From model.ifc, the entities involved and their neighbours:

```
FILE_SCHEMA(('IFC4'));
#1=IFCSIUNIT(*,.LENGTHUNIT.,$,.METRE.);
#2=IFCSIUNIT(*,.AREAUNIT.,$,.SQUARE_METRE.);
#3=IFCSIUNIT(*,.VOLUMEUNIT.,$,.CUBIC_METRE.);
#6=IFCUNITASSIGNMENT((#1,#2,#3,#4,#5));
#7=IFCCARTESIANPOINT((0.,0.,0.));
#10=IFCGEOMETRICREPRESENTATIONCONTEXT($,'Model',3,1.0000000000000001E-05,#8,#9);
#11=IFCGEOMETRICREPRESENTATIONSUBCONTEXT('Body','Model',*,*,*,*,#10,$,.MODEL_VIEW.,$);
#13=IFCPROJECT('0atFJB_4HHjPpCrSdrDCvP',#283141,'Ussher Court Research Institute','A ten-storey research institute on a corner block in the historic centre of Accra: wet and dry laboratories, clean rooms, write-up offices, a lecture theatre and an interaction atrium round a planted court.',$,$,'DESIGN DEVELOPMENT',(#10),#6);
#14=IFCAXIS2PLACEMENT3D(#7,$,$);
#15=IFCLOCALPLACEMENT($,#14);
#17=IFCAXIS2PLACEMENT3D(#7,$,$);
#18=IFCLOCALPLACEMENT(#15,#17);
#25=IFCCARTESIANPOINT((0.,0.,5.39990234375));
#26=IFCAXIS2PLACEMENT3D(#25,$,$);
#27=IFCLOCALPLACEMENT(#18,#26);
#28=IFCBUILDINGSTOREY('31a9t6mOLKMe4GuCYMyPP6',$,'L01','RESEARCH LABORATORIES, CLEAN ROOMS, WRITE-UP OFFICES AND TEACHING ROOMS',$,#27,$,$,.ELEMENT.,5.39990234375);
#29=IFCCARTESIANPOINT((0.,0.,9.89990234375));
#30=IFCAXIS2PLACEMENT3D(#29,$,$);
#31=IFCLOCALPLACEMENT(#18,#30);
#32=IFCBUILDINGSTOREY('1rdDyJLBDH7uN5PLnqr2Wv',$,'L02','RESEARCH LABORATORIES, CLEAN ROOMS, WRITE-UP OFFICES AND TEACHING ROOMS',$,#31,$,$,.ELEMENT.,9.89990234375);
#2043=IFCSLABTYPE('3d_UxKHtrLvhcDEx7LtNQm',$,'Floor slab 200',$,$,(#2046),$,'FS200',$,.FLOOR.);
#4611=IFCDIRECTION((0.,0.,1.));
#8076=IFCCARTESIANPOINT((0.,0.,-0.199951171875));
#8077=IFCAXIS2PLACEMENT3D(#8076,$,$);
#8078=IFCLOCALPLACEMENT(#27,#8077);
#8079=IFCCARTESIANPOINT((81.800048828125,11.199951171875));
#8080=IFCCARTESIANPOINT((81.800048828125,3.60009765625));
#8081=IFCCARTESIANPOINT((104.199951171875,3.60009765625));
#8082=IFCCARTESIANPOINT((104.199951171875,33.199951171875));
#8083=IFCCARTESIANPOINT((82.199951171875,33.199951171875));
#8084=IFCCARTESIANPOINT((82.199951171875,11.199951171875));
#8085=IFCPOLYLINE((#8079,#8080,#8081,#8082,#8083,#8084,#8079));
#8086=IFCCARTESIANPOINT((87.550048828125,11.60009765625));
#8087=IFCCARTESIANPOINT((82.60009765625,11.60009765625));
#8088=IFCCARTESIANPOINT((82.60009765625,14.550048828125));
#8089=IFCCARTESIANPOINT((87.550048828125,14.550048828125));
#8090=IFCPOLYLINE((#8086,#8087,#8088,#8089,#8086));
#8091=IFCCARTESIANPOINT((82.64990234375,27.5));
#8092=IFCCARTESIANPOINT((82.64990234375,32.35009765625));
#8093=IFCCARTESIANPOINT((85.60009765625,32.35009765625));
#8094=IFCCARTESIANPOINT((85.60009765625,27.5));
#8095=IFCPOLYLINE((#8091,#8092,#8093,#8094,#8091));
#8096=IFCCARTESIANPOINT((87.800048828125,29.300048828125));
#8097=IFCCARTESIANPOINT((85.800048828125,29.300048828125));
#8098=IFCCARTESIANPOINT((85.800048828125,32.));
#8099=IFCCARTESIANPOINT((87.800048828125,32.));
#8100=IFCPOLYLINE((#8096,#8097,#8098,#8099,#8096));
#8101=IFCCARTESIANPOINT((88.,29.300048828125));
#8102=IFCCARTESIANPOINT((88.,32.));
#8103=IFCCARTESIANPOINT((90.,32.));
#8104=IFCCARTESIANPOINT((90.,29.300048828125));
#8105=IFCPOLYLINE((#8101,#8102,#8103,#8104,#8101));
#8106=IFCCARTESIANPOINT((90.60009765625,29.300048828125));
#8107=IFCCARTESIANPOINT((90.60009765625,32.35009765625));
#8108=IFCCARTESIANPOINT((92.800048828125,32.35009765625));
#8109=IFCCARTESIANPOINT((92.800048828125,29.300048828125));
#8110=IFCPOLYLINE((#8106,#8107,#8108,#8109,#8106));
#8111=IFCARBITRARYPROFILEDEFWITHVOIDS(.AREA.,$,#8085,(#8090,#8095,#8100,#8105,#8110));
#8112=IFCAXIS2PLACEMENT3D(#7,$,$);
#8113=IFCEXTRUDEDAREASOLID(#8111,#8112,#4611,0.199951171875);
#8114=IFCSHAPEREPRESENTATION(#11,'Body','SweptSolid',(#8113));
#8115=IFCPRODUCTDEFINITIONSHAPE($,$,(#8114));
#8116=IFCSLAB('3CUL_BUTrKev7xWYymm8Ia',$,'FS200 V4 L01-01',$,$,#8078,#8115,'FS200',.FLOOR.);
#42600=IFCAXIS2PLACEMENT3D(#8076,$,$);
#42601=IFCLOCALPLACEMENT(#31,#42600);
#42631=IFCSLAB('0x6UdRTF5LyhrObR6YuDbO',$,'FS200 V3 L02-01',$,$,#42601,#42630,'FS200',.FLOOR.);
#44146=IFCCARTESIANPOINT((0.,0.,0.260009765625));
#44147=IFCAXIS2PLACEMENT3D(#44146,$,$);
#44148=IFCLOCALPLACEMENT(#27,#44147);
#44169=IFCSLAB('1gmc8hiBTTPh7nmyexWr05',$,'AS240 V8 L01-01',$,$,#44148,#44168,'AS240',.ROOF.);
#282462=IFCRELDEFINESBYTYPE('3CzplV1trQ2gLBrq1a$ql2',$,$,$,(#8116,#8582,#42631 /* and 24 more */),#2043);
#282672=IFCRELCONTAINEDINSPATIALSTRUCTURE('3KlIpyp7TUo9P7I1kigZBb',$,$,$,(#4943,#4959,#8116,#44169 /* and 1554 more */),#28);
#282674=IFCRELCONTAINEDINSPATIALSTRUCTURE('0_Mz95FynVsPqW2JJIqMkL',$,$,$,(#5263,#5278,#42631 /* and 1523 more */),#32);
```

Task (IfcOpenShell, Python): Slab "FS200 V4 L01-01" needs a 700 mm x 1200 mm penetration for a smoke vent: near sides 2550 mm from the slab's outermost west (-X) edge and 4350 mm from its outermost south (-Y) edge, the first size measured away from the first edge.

```python
import numpy as np
import ifcopenshell
import ifcopenshell.api.feature
import ifcopenshell.api.geometry
import ifcopenshell.api.root
import ifcopenshell.geom
import ifcopenshell.util.placement
import ifcopenshell.util.representation
import ifcopenshell.util.shape
import ifcopenshell.util.unit

model = ifcopenshell.open("model.ifc")
unit_scale = ifcopenshell.util.unit.calculate_unit_scale(model)
settings = ifcopenshell.geom.settings()


def volume(element):
    """Net volume in cubic metres, openings subtracted."""
    shape = ifcopenshell.geom.create_shape(settings, element)
    return ifcopenshell.util.shape.get_volume(shape.geometry)


slab = model.by_guid("3CUL_BUTrKev7xWYymm8Ia")
before = volume(slab)

# Extent in the slab's own axes, in metres. The edges named are its -X and -Y sides.
slab_shape = ifcopenshell.geom.create_shape(settings, slab)
vertices = ifcopenshell.util.shape.get_vertices(slab_shape.geometry)
x_min, y_min, bottom = vertices.min(axis=0)
top = vertices[:, 2].max()

opening = ifcopenshell.api.root.create_entity(model, ifc_class="IfcOpeningElement", name="Smoke vent opening", predefined_type="OPENING")
context = ifcopenshell.util.representation.get_context(model, "Model", "Body", "MODEL_VIEW")
width, depth = 0.7, 1.2
outline = [(0.0, 0.0), (width, 0.0), (width, depth), (0.0, depth), (0.0, 0.0)]
# Overshoot both faces by 50 mm so the cut is clean.
shape = ifcopenshell.api.geometry.add_slab_representation(
    model, context=context, depth=top - bottom + 0.1, polyline=outline
)
ifcopenshell.api.geometry.assign_representation(model, product=opening, representation=shape)

matrix = ifcopenshell.util.placement.get_local_placement(slab.ObjectPlacement)
matrix[:, 3] = matrix @ np.append(np.array([x_min + 2.55, y_min + 4.35, bottom - 0.05]) / unit_scale, 1.0)
ifcopenshell.api.geometry.edit_object_placement(model, product=opening, matrix=matrix, is_si=False)
ifcopenshell.api.feature.add_feature(model, feature=opening, element=slab)

after = volume(slab)

print(f"slab volume {before:.3f} -> {after:.3f} m3")

model.write("model_updated.ifc")
```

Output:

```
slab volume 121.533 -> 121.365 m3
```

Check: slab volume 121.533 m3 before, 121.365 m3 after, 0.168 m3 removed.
